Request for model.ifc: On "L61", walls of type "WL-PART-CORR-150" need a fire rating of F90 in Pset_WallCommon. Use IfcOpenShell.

First a look at what the model holds.

```python
import ifcopenshell
import ifcopenshell.util.element

model = ifcopenshell.open("model.ifc")
print(model.schema)
storey = next(s for s in model.by_type("IfcBuildingStorey") if s.Name == "L61")
walls = [e for e in ifcopenshell.util.element.get_decomposition(storey) if e.is_a("IfcWall")]
seen = {}
for e in walls:
    element_type = ifcopenshell.util.element.get_type(e)
    key = (element_type.Name if element_type != e and element_type else None, ifcopenshell.util.element.get_pset(e, "Pset_WallCommon", "FireRating"))
    seen[key] = seen.get(key, 0) + 1
for (name, value), count in sorted(seen.items(), key=str):
    print(count, "x", name, "|", value)
```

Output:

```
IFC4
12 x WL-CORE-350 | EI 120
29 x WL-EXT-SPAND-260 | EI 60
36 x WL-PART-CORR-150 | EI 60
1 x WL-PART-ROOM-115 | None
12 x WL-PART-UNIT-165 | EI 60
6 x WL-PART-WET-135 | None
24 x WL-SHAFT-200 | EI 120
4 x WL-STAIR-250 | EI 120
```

```python
import ifcopenshell
import ifcopenshell.api.pset
import ifcopenshell.util.element

model = ifcopenshell.open("model.ifc")

storey = next(s for s in model.by_type("IfcBuildingStorey") if s.Name == "L61")
walls = [e for e in ifcopenshell.util.element.get_decomposition(storey) if e.is_a("IfcWall")]

count = 0
for e in walls:
    element_type = ifcopenshell.util.element.get_type(e)
    if element_type in (None, e) or element_type.Name != "WL-PART-CORR-150":
        continue
    found = ifcopenshell.util.element.get_pset(e, "Pset_WallCommon", should_inherit=False)
    if found:
        pset = model.by_id(found["id"])
        if len(ifcopenshell.util.element.get_elements_by_pset(pset)) > 1:
            pset = ifcopenshell.api.pset.unshare_pset(model, products=[e], pset=pset)[0]
    else:
        pset = ifcopenshell.api.pset.add_pset(model, product=e, name="Pset_WallCommon")
    ifcopenshell.api.pset.edit_pset(model, pset=pset, properties={"FireRating": "F90"})
    count += 1

print(count, "walls updated")

model.write("model_updated.ifc")
```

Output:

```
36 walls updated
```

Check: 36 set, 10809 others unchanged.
